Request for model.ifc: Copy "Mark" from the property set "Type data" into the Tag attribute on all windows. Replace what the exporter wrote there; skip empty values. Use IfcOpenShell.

First a look at what the model holds.

```python
import ifcopenshell
import ifcopenshell.util.element

model = ifcopenshell.open("model.ifc")
print(model.schema)
windows = model.by_type("IfcWindow")
print(len(windows), "windows")
for e in windows[:8]:
    source = ifcopenshell.util.element.get_pset(e, "Type data", "Mark")
    target = e.Tag
    print(e.id(), repr(source), repr(target), sep=" | ")
```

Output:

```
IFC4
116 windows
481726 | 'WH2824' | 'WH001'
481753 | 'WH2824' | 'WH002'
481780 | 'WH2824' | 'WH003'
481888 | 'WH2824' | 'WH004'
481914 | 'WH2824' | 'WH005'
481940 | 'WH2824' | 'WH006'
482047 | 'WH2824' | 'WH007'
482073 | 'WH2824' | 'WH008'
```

```python
import ifcopenshell
import ifcopenshell.util.element

model = ifcopenshell.open("model.ifc")

count = 0
for e in model.by_type("IfcWindow"):
    value = ifcopenshell.util.element.get_pset(e, "Type data", "Mark")
    current = e.Tag
    if not value or not value.strip() or current == value:
        continue
    e.Tag = value
    count += 1

print(count, "windows updated")

model.write("model_rev.ifc")
```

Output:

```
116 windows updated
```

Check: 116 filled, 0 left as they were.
